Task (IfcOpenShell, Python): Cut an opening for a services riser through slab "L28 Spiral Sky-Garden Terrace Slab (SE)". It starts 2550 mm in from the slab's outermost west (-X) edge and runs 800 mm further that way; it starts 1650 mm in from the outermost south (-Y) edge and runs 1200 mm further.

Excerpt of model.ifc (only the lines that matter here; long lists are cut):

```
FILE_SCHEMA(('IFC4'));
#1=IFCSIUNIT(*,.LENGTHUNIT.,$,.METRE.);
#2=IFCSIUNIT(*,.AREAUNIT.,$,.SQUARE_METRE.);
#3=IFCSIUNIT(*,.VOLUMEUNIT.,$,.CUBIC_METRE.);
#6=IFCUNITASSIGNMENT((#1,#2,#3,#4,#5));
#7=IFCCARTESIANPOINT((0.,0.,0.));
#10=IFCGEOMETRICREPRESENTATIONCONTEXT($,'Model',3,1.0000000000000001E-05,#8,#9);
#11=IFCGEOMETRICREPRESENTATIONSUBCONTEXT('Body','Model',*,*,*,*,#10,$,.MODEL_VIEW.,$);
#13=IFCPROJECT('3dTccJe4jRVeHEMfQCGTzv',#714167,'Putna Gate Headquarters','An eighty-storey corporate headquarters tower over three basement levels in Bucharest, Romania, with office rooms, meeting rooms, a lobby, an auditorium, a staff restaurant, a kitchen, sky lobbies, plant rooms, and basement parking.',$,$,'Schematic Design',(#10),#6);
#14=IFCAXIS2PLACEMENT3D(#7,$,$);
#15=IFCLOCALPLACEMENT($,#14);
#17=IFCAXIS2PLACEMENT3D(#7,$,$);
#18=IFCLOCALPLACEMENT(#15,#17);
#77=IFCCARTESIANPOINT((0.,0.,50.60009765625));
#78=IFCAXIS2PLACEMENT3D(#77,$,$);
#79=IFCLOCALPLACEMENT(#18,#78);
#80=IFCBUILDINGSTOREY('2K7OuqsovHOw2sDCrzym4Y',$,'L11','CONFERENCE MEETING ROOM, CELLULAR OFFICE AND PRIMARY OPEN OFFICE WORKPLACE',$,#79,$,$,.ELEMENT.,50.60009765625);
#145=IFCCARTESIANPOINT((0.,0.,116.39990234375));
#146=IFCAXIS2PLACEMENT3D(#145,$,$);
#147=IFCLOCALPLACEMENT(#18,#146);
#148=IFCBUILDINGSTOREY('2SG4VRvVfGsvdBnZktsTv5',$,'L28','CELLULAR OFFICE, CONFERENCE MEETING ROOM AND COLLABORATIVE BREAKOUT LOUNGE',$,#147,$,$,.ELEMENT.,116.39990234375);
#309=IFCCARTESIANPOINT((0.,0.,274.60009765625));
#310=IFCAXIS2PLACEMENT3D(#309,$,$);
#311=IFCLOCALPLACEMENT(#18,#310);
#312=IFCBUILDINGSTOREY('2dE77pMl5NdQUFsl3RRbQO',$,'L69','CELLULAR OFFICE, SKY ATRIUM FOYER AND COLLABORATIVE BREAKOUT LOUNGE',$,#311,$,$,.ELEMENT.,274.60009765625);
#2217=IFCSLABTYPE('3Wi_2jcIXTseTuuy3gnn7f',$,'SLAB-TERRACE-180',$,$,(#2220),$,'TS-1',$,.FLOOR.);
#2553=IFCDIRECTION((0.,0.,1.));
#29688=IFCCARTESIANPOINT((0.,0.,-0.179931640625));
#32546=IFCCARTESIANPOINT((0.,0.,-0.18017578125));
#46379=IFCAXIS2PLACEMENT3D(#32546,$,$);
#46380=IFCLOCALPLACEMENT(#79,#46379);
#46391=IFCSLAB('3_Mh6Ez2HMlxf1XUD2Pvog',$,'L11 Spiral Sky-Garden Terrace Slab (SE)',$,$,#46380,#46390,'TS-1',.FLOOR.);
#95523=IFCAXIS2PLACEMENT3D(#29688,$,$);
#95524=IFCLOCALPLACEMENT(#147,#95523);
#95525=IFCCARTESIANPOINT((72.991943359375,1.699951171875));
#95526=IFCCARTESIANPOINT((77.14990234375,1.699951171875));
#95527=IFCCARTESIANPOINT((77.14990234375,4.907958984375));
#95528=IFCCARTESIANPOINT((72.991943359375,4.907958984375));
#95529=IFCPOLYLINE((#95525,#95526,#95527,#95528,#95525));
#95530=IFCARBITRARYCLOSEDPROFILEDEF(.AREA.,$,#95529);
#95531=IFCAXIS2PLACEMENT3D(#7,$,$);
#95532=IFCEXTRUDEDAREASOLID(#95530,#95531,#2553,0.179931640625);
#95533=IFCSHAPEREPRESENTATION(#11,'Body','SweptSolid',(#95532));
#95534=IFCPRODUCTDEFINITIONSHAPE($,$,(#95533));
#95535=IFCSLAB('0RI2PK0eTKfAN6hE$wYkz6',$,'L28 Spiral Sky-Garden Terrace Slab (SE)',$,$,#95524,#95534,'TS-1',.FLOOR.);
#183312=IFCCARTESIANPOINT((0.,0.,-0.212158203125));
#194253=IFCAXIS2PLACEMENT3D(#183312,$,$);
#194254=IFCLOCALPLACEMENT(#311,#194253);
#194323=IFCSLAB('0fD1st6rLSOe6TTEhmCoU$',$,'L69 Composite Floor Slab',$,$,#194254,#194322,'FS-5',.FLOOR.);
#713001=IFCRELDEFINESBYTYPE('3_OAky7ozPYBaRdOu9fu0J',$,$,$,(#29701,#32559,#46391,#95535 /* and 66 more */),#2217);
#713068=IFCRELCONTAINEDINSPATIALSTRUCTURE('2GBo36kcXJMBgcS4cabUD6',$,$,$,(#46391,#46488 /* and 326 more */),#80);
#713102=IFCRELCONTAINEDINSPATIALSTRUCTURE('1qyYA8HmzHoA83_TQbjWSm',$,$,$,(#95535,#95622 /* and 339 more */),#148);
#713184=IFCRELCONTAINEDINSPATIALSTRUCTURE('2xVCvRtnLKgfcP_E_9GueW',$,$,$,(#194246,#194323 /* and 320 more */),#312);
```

```python
import numpy as np
import ifcopenshell
import ifcopenshell.api.feature
import ifcopenshell.api.geometry
import ifcopenshell.api.root
import ifcopenshell.geom
import ifcopenshell.util.placement
import ifcopenshell.util.representation
import ifcopenshell.util.shape
import ifcopenshell.util.unit

model = ifcopenshell.open("model.ifc")
unit_scale = ifcopenshell.util.unit.calculate_unit_scale(model)
settings = ifcopenshell.geom.settings()


def volume(element):
    """Net volume in cubic metres, openings subtracted."""
    shape = ifcopenshell.geom.create_shape(settings, element)
    return ifcopenshell.util.shape.get_volume(shape.geometry)


slab = model.by_guid("0RI2PK0eTKfAN6hE$wYkz6")
before = volume(slab)

# Extent in the slab's own axes, in metres. The edges named are its -X and -Y sides.
slab_shape = ifcopenshell.geom.create_shape(settings, slab)
vertices = ifcopenshell.util.shape.get_vertices(slab_shape.geometry)
x_min, y_min, bottom = vertices.min(axis=0)
top = vertices[:, 2].max()

opening = ifcopenshell.api.root.create_entity(model, ifc_class="IfcOpeningElement", name="Services riser opening", predefined_type="OPENING")
context = ifcopenshell.util.representation.get_context(model, "Model", "Body", "MODEL_VIEW")
width, depth = 0.8, 1.2
outline = [(0.0, 0.0), (width, 0.0), (width, depth), (0.0, depth), (0.0, 0.0)]
# Overshoot both faces by 50 mm so the cut is clean.
shape = ifcopenshell.api.geometry.add_slab_representation(
    model, context=context, depth=top - bottom + 0.1, polyline=outline
)
ifcopenshell.api.geometry.assign_representation(model, product=opening, representation=shape)

matrix = ifcopenshell.util.placement.get_local_placement(slab.ObjectPlacement)
matrix[:, 3] = matrix @ np.append(np.array([x_min + 2.55, y_min + 1.65, bottom - 0.05]) / unit_scale, 1.0)
ifcopenshell.api.geometry.edit_object_placement(model, product=opening, matrix=matrix, is_si=False)
ifcopenshell.api.feature.add_feature(model, feature=opening, element=slab)

after = volume(slab)

print(f"slab volume {before:.3f} -> {after:.3f} m3")

model.write("model_v2.ifc")
```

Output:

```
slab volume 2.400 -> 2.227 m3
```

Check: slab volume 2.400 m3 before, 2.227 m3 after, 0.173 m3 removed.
